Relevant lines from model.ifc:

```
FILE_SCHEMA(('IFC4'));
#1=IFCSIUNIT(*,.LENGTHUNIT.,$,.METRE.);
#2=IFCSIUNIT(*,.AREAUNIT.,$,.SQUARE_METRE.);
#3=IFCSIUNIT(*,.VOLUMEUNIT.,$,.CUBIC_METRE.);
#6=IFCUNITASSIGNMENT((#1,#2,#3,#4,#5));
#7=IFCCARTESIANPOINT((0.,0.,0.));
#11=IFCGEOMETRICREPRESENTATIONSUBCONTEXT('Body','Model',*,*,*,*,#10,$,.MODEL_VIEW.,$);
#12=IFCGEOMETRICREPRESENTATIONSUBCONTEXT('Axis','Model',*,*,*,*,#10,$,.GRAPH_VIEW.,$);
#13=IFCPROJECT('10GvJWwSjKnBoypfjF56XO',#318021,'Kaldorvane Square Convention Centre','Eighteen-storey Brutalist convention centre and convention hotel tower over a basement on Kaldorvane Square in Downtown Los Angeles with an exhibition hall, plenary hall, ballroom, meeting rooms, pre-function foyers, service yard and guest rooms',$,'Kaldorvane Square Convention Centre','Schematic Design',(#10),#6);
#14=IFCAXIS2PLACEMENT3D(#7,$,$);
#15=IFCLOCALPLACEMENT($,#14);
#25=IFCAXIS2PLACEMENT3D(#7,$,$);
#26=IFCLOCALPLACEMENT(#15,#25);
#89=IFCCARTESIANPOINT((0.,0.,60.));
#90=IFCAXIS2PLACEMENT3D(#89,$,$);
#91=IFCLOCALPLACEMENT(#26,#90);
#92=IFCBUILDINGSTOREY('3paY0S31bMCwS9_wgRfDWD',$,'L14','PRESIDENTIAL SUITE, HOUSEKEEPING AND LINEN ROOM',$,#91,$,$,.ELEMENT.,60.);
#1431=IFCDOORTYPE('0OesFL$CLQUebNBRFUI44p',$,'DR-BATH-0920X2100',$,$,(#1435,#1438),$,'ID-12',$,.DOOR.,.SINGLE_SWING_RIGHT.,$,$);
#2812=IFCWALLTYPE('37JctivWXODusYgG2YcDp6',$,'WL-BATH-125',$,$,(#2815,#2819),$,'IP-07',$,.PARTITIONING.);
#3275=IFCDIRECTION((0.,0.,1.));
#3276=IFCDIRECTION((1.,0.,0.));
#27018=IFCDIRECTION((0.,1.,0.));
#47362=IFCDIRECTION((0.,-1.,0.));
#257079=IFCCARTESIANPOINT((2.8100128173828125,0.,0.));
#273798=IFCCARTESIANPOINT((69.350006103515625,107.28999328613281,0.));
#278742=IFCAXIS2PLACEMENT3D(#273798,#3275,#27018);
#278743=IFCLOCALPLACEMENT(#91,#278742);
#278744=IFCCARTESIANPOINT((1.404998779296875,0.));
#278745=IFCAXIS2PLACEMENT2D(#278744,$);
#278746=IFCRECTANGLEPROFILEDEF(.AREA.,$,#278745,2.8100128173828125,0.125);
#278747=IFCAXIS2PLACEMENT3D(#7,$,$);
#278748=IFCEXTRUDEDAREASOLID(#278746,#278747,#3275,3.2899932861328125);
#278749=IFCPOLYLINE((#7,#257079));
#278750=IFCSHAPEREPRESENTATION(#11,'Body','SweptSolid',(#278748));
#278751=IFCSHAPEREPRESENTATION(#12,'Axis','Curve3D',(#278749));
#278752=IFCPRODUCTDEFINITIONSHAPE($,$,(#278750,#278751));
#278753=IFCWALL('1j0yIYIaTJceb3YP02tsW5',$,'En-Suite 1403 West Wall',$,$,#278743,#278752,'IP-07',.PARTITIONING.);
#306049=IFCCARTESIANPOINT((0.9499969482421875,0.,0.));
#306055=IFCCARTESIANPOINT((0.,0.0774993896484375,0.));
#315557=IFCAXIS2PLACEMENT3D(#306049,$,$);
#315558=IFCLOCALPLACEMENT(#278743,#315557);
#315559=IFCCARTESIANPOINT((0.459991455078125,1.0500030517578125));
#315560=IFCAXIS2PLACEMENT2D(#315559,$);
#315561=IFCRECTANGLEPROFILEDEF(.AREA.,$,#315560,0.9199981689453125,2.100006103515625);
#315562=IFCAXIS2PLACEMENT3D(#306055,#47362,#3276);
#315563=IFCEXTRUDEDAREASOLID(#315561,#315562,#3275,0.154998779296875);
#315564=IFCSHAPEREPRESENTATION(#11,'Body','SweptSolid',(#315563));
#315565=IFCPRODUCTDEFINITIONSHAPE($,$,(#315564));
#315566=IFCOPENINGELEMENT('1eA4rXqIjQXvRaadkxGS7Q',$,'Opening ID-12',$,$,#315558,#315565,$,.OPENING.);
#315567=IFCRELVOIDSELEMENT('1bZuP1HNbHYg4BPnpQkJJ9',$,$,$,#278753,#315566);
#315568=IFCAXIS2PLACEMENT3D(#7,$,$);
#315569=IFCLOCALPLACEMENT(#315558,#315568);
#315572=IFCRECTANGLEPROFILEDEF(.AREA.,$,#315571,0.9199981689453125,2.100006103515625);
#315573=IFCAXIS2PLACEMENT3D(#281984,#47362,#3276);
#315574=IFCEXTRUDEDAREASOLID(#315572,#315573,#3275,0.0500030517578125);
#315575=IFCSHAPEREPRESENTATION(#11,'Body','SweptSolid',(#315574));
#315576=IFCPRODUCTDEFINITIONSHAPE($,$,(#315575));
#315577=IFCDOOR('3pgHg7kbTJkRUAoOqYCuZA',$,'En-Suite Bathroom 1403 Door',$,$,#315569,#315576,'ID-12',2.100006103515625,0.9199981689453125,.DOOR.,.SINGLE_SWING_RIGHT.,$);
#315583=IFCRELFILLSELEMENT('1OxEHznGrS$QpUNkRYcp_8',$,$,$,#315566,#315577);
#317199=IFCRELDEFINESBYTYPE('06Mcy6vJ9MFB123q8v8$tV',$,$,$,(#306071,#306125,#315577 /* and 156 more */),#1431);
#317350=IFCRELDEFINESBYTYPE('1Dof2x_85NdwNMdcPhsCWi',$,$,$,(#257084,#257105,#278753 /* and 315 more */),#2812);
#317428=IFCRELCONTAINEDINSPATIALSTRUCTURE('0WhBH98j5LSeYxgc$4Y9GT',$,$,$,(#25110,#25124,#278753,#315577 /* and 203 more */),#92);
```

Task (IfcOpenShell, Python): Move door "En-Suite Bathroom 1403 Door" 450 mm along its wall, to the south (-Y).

```python
import ifcopenshell
import ifcopenshell.api.geometry
import ifcopenshell.util.placement

model = ifcopenshell.open("model.ifc")

door = model.by_guid("3pgHg7kbTJkRUAoOqYCuZA")
opening = door.FillsVoids[0].RelatingOpeningElement
wall = opening.VoidsElements[0].RelatingBuildingElement

wall_matrix = ifcopenshell.util.placement.get_local_placement(wall.ObjectPlacement)
shift = wall_matrix[:3, 0] * -0.45
before = ifcopenshell.util.placement.get_local_placement(door.ObjectPlacement)[:3, 3].copy()

# The door is placed relative to its opening, so it follows when the opening moves.
matrix = ifcopenshell.util.placement.get_local_placement(opening.ObjectPlacement)
matrix[:3, 3] += shift
ifcopenshell.api.geometry.edit_object_placement(
    model, product=opening, matrix=matrix, is_si=False, should_transform_children=True
)

after = ifcopenshell.util.placement.get_local_placement(door.ObjectPlacement)[:3, 3]
print("door moved by", (after - before).round(3) + 0.0)

model.write("model-out.ifc")
```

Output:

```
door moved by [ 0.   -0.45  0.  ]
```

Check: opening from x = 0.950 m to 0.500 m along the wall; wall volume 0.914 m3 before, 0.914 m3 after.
